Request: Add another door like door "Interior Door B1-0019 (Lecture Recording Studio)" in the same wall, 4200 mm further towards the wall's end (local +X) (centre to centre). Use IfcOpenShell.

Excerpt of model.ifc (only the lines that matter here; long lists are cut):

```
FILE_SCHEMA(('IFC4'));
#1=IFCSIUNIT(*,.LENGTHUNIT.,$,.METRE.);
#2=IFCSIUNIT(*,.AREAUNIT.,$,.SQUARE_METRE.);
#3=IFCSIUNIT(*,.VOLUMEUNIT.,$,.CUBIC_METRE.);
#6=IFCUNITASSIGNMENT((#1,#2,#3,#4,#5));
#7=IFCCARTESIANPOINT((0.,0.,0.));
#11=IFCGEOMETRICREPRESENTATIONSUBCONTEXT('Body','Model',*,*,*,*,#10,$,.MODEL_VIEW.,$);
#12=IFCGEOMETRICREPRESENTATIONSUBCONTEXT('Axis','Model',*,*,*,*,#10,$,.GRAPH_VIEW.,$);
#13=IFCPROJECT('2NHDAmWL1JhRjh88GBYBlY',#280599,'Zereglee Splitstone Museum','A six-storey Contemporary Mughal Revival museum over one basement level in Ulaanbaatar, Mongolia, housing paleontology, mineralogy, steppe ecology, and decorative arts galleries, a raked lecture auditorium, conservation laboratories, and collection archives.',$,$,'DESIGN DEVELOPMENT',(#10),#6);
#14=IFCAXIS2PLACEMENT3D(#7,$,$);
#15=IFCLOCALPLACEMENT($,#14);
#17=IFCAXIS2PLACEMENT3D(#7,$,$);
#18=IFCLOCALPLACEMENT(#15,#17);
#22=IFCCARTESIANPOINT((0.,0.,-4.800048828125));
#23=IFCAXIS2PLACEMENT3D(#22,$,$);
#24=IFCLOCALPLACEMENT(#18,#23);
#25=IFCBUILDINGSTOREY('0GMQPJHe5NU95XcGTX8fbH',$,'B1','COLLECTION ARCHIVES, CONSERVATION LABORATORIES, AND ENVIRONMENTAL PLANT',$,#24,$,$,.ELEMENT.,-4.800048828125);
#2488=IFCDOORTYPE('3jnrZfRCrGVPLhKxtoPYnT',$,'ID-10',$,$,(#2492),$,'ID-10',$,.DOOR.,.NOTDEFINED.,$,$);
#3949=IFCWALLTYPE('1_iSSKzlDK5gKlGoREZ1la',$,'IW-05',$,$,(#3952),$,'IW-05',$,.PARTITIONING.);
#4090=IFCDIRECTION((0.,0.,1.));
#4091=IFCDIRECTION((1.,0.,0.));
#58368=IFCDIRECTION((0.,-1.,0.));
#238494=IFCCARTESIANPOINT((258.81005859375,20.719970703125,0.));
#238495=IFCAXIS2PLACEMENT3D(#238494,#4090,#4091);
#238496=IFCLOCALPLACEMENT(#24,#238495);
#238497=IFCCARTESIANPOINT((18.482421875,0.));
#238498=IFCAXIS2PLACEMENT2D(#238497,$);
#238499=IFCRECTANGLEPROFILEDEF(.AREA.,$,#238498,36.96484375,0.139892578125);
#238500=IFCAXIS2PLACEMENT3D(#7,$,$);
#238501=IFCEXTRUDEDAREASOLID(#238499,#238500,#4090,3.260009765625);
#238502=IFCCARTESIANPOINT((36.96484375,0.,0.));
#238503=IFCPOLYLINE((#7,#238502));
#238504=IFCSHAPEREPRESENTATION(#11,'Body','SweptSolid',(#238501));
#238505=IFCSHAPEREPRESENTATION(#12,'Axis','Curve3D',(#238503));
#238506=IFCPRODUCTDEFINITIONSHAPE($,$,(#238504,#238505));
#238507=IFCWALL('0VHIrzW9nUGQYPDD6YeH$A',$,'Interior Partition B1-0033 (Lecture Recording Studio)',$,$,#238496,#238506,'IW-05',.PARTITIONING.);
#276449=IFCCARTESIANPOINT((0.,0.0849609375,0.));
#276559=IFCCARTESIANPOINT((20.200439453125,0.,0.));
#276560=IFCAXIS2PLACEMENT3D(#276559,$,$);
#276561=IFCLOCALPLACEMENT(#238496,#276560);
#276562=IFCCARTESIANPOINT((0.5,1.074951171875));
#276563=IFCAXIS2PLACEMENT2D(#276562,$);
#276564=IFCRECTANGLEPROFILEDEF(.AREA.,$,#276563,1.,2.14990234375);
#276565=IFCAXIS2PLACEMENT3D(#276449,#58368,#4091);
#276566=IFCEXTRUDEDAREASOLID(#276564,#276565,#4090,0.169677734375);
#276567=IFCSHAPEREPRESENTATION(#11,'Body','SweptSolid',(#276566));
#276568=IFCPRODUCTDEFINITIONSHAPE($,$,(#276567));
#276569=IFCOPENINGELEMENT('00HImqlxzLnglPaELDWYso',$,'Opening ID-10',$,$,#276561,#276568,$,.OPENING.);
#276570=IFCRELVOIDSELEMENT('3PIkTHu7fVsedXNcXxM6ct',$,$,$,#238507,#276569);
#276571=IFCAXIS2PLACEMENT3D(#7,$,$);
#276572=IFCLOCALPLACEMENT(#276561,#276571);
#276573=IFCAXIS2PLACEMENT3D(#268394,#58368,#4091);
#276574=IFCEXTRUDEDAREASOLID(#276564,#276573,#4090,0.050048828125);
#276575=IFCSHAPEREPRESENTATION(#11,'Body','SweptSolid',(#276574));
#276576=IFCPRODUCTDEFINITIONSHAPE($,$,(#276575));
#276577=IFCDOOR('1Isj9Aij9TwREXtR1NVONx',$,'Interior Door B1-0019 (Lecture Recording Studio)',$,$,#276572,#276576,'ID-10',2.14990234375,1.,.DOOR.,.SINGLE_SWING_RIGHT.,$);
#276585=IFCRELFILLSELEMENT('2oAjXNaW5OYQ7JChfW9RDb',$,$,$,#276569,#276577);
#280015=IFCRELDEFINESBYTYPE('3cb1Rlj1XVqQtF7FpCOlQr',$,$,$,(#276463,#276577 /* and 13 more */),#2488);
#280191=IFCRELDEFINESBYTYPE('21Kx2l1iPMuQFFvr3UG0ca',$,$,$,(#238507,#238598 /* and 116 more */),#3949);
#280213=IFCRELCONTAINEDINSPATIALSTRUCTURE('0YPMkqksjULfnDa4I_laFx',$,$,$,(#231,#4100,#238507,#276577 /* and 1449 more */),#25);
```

```python
import ifcopenshell
import ifcopenshell.api.feature
import ifcopenshell.api.geometry
import ifcopenshell.api.root
import ifcopenshell.geom
import ifcopenshell.util.element
import ifcopenshell.util.placement
import ifcopenshell.util.shape

model = ifcopenshell.open("model.ifc")
settings = ifcopenshell.geom.settings()


def volume(element):
    """Net volume in cubic metres, openings subtracted."""
    shape = ifcopenshell.geom.create_shape(settings, element)
    return ifcopenshell.util.shape.get_volume(shape.geometry)


door = model.by_guid("1Isj9Aij9TwREXtR1NVONx")
opening = door.FillsVoids[0].RelatingOpeningElement
wall = opening.VoidsElements[0].RelatingBuildingElement
before = volume(wall)
shift = ifcopenshell.util.placement.get_local_placement(wall.ObjectPlacement)[:3, 0] * 4.2

# copy_class copies the void relationship, type, container and properties, but no geometry.
new_opening = ifcopenshell.api.root.copy_class(model, product=opening)
new_opening.Representation = ifcopenshell.util.element.copy_deep(
    model, opening.Representation, exclude=["IfcGeometricRepresentationContext", "IfcRepresentationMap"]
)
new_door = ifcopenshell.api.root.copy_class(model, product=door)
new_door.Representation = ifcopenshell.util.element.copy_deep(
    model, door.Representation, exclude=["IfcGeometricRepresentationContext", "IfcRepresentationMap"]
)
new_door.Tag = None
ifcopenshell.api.feature.add_filling(model, opening=new_opening, element=new_door)

for old, new in ((opening, new_opening), (door, new_door)):
    matrix = ifcopenshell.util.placement.get_local_placement(old.ObjectPlacement)
    matrix[:3, 3] += shift
    ifcopenshell.api.geometry.edit_object_placement(model, product=new, matrix=matrix, is_si=False)

after = volume(wall)

print(f"wall volume {before:.3f} -> {after:.3f} m3")

model.write("model_updated.ifc")
```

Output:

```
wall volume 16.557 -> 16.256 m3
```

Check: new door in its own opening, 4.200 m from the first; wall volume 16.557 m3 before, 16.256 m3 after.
